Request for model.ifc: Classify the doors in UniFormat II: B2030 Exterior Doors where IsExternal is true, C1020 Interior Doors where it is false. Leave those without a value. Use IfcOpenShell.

First a look at what the model holds.

```python
import ifcopenshell
import ifcopenshell.util.element

model = ifcopenshell.open("model.ifc")
print(model.schema)
print("classifications:", [c.Name for c in model.by_type("IfcClassification")])
values = [ifcopenshell.util.element.get_pset(e, "Pset_DoorCommon", "IsExternal") for e in model.by_type("IfcDoor")]
for value in (True, False, None):
    print("IsExternal", value, values.count(value))
```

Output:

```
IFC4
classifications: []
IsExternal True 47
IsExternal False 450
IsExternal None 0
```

```python
import ifcopenshell
import ifcopenshell.api.classification
import ifcopenshell.util.element

model = ifcopenshell.open("model.ifc")

system = ifcopenshell.api.classification.add_classification(model, classification="UniFormat II")

doors = model.by_type("IfcDoor")
external = {e: ifcopenshell.util.element.get_pset(e, "Pset_DoorCommon", "IsExternal") for e in doors}
for flag, code, name in ((True, "B2030", "Exterior Doors"), (False, "C1020", "Interior Doors")):
    products = [e for e in doors if external[e] is flag]
    ifcopenshell.api.classification.add_reference(
        model, products=products, classification=system, identification=code, name=name
    )
    print(code, len(products))

model.write("model-out.ifc")
```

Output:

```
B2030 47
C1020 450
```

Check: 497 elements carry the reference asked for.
